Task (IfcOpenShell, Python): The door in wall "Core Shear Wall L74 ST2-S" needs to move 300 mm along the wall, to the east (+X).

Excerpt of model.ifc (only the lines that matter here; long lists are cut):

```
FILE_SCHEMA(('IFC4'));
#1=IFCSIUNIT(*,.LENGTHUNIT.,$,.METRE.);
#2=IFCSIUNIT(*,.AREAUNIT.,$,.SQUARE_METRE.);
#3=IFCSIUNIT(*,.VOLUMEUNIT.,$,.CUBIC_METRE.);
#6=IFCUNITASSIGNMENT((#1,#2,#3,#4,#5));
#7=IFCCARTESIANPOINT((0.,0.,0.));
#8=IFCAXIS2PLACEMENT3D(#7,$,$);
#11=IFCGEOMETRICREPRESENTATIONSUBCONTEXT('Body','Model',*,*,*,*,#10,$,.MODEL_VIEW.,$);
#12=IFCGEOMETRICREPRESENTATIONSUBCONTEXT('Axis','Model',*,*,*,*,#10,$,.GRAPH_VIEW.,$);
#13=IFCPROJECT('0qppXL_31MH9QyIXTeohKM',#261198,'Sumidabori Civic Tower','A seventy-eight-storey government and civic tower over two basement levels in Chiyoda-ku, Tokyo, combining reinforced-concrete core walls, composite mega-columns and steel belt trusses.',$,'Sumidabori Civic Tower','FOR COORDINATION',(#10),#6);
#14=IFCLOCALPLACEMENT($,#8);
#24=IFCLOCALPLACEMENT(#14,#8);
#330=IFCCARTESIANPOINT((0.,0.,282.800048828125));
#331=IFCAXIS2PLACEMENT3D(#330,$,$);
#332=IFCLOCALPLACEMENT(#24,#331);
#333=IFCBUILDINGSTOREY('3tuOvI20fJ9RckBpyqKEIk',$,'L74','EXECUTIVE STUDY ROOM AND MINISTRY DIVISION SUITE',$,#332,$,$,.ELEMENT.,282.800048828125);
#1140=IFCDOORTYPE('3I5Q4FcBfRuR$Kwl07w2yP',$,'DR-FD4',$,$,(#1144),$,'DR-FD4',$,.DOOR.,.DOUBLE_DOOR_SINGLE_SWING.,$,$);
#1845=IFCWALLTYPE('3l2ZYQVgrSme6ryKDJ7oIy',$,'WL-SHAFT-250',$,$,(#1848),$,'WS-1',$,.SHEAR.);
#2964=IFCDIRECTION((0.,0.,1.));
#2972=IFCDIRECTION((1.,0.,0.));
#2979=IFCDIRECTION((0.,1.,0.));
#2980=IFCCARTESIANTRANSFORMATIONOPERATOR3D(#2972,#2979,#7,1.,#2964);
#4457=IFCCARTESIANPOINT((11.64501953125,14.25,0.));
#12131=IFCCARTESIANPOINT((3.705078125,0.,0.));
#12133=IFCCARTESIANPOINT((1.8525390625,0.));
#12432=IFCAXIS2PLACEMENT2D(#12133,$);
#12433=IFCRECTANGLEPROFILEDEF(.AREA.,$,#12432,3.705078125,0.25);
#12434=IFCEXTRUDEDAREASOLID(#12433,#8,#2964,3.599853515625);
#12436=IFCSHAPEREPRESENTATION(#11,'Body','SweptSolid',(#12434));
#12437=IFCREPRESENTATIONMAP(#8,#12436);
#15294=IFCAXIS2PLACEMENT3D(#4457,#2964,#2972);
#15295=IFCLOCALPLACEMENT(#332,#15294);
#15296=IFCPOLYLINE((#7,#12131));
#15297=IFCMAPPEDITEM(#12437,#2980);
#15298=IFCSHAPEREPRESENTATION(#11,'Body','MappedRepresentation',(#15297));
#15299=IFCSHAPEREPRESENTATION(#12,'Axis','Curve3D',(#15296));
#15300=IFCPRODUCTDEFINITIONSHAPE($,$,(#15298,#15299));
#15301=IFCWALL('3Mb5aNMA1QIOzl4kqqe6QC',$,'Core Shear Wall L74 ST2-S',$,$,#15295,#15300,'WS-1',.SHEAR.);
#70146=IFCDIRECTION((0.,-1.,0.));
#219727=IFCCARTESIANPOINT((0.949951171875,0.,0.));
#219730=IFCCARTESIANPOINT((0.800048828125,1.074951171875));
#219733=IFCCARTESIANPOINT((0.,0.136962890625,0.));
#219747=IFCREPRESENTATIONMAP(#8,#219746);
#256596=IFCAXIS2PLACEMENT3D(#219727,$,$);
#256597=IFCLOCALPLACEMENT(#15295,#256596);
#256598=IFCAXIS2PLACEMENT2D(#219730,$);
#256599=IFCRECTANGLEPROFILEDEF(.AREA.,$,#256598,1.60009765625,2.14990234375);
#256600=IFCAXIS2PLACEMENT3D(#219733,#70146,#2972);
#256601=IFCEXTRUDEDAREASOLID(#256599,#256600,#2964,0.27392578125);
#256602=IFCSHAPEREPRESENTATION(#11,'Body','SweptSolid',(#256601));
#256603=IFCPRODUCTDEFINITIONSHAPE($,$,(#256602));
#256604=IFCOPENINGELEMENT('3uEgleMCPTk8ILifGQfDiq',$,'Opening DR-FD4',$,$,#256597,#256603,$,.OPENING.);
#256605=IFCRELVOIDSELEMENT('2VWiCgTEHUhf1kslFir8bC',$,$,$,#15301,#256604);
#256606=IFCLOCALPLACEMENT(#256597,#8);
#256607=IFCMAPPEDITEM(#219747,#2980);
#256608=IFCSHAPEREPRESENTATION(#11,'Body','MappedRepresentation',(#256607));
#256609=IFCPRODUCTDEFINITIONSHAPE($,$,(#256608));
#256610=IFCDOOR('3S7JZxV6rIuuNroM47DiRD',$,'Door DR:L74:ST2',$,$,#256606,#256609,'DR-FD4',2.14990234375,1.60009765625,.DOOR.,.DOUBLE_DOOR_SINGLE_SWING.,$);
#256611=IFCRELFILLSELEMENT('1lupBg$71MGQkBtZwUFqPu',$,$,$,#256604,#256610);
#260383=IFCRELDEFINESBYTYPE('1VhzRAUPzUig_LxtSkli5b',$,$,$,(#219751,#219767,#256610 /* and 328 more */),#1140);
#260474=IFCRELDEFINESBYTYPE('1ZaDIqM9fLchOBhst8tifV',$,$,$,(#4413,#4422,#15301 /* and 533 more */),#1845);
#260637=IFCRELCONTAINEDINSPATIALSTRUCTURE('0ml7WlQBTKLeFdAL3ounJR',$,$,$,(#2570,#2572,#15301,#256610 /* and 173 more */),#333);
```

```python
import ifcopenshell
import ifcopenshell.api.geometry
import ifcopenshell.util.placement
import ifcopenshell.util.unit

model = ifcopenshell.open("model.ifc")
unit_scale = ifcopenshell.util.unit.calculate_unit_scale(model)

door = model.by_guid("3S7JZxV6rIuuNroM47DiRD")
opening = door.FillsVoids[0].RelatingOpeningElement
wall = opening.VoidsElements[0].RelatingBuildingElement

wall_matrix = ifcopenshell.util.placement.get_local_placement(wall.ObjectPlacement)
shift = wall_matrix[:3, 0] * 0.3 / unit_scale
before = ifcopenshell.util.placement.get_local_placement(door.ObjectPlacement)[:3, 3].copy()

# The door is placed relative to its opening, so it follows when the opening moves.
matrix = ifcopenshell.util.placement.get_local_placement(opening.ObjectPlacement)
matrix[:3, 3] += shift
ifcopenshell.api.geometry.edit_object_placement(
    model, product=opening, matrix=matrix, is_si=False, should_transform_children=True
)

after = ifcopenshell.util.placement.get_local_placement(door.ObjectPlacement)[:3, 3]
print("door moved by", (after - before).round(3) + 0.0)

model.write("model_edited.ifc")
```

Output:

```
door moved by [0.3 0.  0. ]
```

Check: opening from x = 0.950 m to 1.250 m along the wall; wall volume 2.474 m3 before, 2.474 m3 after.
